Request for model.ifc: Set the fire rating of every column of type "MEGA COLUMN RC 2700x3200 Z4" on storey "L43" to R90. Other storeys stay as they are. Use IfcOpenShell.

First a look at what the model holds.

```python
import ifcopenshell
import ifcopenshell.util.element

model = ifcopenshell.open("model.ifc")
print(model.schema)
storey = next(s for s in model.by_type("IfcBuildingStorey") if s.Name == "L43")
columns = [e for e in ifcopenshell.util.element.get_decomposition(storey) if e.is_a("IfcColumn")]
seen = {}
for e in columns:
    element_type = ifcopenshell.util.element.get_type(e)
    key = (element_type.Name if element_type != e and element_type else None, ifcopenshell.util.element.get_pset(e, "Pset_ColumnCommon", "FireRating"))
    seen[key] = seen.get(key, 0) + 1
for (name, value), count in sorted(seen.items(), key=str):
    print(count, "x", name, "|", value)
```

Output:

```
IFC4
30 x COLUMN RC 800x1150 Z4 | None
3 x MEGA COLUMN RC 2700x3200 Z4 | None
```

```python
import ifcopenshell
import ifcopenshell.api.pset
import ifcopenshell.util.element

model = ifcopenshell.open("model.ifc")

storey = next(s for s in model.by_type("IfcBuildingStorey") if s.Name == "L43")
columns = [e for e in ifcopenshell.util.element.get_decomposition(storey) if e.is_a("IfcColumn")]

count = 0
for e in columns:
    element_type = ifcopenshell.util.element.get_type(e)
    if element_type in (None, e) or element_type.Name != "MEGA COLUMN RC 2700x3200 Z4":
        continue
    # add_pset returns the element's existing set when there is one.
    pset = ifcopenshell.api.pset.add_pset(model, product=e, name="Pset_ColumnCommon")
    ifcopenshell.api.pset.edit_pset(model, pset=pset, properties={"FireRating": "R90"})
    count += 1

print(count, "columns updated")

model.write("model_rev.ifc")
```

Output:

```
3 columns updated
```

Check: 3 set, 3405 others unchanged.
